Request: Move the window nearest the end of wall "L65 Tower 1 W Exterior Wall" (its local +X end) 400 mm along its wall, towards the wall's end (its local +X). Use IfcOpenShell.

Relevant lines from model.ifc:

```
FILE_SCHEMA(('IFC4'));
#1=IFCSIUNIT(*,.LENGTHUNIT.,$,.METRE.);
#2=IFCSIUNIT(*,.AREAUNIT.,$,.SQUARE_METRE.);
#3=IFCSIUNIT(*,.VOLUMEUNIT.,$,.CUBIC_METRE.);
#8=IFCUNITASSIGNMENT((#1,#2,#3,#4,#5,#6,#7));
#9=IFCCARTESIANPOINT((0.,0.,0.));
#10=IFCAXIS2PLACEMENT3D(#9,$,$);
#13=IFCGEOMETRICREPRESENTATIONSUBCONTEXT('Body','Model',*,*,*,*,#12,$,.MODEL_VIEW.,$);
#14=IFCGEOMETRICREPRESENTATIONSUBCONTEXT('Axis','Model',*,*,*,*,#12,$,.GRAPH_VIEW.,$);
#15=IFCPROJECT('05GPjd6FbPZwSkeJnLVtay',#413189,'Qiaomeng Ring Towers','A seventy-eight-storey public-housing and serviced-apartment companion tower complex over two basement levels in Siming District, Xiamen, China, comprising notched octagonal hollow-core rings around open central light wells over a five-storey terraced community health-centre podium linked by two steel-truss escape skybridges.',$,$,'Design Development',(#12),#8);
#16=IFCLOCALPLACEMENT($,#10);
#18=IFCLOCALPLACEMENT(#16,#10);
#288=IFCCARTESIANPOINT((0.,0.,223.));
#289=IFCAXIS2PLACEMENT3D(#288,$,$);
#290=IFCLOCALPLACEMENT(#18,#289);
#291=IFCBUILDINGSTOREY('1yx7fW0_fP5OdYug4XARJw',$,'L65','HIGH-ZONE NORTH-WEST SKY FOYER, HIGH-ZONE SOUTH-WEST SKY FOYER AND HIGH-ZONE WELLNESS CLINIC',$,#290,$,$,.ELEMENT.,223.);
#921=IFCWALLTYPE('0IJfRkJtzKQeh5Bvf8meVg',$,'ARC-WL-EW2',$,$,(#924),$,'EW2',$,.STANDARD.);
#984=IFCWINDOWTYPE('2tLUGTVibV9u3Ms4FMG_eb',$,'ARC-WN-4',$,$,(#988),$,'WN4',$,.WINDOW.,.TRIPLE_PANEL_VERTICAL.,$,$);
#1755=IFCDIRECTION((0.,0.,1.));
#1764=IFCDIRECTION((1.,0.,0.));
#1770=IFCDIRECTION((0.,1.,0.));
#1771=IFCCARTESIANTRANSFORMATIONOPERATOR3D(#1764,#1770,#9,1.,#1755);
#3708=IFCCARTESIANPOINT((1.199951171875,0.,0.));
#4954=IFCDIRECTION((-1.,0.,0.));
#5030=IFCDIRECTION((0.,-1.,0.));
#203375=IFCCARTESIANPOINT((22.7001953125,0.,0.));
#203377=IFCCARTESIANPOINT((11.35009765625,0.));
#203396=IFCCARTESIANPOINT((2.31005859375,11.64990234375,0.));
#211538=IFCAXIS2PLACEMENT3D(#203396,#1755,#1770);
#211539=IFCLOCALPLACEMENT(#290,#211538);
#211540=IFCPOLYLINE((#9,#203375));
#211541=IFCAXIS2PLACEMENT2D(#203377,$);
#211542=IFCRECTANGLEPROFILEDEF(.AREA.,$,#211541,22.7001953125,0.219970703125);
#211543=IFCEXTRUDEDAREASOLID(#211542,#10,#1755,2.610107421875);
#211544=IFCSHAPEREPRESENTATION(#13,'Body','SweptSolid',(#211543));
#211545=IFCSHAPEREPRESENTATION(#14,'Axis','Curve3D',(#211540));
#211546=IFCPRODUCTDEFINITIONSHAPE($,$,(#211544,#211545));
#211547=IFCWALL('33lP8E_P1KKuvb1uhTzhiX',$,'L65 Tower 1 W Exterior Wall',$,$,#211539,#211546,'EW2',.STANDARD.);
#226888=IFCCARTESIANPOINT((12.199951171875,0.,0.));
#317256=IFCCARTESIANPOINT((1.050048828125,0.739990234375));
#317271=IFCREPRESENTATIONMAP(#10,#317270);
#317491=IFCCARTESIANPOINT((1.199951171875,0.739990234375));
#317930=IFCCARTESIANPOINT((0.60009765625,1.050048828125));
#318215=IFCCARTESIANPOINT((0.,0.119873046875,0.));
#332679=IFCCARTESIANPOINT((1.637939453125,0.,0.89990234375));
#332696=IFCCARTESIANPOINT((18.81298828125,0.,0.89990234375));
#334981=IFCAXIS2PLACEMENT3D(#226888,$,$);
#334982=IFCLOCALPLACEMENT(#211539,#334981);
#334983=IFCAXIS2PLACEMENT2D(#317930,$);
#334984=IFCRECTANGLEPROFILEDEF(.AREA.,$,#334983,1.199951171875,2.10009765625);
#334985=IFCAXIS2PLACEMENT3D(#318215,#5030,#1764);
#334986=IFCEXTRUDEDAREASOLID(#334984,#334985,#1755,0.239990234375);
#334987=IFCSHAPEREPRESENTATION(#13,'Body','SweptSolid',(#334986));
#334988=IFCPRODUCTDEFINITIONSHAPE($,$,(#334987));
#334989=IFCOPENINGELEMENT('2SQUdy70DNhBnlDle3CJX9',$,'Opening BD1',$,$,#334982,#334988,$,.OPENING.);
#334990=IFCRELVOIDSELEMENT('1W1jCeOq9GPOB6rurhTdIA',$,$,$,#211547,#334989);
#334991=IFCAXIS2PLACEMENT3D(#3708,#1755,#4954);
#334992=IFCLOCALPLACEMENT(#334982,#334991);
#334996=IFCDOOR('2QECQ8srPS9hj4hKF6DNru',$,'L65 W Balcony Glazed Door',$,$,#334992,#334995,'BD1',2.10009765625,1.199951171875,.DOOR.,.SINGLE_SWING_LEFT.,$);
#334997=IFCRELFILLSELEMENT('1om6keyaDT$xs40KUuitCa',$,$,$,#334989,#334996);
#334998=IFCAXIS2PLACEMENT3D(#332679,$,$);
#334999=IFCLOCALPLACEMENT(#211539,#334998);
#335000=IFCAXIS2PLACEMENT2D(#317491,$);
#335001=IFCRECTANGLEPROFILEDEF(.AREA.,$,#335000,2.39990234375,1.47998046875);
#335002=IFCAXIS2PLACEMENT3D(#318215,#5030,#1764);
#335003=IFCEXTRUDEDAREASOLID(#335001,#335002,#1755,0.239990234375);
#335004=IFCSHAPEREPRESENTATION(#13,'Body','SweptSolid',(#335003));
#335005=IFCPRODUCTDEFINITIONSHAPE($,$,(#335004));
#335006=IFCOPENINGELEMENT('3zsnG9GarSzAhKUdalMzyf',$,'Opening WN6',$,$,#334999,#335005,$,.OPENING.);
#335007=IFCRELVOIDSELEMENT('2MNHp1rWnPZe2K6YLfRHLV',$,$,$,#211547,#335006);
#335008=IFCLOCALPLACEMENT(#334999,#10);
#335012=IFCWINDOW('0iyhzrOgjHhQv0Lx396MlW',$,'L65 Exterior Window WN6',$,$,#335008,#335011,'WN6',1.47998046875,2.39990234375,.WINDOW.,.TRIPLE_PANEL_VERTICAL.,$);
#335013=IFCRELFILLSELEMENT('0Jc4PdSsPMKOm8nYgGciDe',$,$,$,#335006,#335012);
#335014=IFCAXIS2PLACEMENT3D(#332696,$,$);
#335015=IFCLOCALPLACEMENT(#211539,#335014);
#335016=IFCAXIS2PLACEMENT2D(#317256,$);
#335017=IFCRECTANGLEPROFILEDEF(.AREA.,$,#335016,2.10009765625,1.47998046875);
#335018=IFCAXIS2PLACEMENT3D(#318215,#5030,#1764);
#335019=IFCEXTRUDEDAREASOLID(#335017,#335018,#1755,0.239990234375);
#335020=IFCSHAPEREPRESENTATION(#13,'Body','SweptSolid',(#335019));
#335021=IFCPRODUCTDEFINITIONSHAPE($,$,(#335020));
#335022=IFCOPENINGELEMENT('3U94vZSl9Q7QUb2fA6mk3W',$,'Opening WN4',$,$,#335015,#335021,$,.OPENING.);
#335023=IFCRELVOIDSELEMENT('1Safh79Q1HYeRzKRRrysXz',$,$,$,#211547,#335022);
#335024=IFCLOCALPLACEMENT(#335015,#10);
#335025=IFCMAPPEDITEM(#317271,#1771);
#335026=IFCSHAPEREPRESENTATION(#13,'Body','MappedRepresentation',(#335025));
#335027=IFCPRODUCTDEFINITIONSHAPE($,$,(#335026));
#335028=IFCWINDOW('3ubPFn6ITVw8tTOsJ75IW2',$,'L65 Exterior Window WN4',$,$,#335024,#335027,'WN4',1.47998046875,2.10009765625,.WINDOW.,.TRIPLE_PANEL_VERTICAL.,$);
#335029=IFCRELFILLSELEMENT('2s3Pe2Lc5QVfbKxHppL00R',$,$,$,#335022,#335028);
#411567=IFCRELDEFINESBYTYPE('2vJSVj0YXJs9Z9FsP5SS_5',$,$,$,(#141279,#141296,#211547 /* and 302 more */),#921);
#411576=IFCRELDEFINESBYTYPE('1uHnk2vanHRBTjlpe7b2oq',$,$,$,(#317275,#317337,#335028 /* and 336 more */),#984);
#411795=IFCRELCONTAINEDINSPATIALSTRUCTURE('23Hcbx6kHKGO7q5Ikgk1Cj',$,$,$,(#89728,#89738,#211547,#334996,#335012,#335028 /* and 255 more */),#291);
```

```python
import ifcopenshell
import ifcopenshell.api.geometry
import ifcopenshell.util.placement
import ifcopenshell.util.unit

model = ifcopenshell.open("model.ifc")
unit_scale = ifcopenshell.util.unit.calculate_unit_scale(model)

window = model.by_id(335028)
opening = window.FillsVoids[0].RelatingOpeningElement
wall = opening.VoidsElements[0].RelatingBuildingElement

wall_matrix = ifcopenshell.util.placement.get_local_placement(wall.ObjectPlacement)
shift = wall_matrix[:3, 0] * 0.4 / unit_scale
before = ifcopenshell.util.placement.get_local_placement(window.ObjectPlacement)[:3, 3].copy()

# The window is placed relative to its opening, so it follows when the opening moves.
matrix = ifcopenshell.util.placement.get_local_placement(opening.ObjectPlacement)
matrix[:3, 3] += shift
ifcopenshell.api.geometry.edit_object_placement(
    model, product=opening, matrix=matrix, is_si=False, should_transform_children=True
)

after = ifcopenshell.util.placement.get_local_placement(window.ObjectPlacement)[:3, 3]
print("window moved by", (after - before).round(3) + 0.0)

model.write("model_rev.ifc")
```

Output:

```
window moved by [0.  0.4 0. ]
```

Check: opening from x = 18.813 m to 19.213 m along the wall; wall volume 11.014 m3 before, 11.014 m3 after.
